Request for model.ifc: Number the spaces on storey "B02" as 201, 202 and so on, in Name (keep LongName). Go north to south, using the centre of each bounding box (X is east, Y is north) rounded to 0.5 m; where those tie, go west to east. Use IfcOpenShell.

First a look at what the model holds.

```python
import ifcopenshell
import ifcopenshell.util.element
import ifcopenshell.util.placement

model = ifcopenshell.open("model.ifc")
print(model.schema)
storey = next(s for s in model.by_type("IfcBuildingStorey") if s.Name == "B02")
spaces = [e for e in ifcopenshell.util.element.get_decomposition(storey) if e.is_a("IfcSpace")]
for e in sorted(spaces, key=lambda e: e.id()):
    origin = ifcopenshell.util.placement.get_local_placement(e.ObjectPlacement)[:3, 3]
    print(e.id(), e.Name, e.LongName, origin.round(2) + 0.0, sep=" | ")
```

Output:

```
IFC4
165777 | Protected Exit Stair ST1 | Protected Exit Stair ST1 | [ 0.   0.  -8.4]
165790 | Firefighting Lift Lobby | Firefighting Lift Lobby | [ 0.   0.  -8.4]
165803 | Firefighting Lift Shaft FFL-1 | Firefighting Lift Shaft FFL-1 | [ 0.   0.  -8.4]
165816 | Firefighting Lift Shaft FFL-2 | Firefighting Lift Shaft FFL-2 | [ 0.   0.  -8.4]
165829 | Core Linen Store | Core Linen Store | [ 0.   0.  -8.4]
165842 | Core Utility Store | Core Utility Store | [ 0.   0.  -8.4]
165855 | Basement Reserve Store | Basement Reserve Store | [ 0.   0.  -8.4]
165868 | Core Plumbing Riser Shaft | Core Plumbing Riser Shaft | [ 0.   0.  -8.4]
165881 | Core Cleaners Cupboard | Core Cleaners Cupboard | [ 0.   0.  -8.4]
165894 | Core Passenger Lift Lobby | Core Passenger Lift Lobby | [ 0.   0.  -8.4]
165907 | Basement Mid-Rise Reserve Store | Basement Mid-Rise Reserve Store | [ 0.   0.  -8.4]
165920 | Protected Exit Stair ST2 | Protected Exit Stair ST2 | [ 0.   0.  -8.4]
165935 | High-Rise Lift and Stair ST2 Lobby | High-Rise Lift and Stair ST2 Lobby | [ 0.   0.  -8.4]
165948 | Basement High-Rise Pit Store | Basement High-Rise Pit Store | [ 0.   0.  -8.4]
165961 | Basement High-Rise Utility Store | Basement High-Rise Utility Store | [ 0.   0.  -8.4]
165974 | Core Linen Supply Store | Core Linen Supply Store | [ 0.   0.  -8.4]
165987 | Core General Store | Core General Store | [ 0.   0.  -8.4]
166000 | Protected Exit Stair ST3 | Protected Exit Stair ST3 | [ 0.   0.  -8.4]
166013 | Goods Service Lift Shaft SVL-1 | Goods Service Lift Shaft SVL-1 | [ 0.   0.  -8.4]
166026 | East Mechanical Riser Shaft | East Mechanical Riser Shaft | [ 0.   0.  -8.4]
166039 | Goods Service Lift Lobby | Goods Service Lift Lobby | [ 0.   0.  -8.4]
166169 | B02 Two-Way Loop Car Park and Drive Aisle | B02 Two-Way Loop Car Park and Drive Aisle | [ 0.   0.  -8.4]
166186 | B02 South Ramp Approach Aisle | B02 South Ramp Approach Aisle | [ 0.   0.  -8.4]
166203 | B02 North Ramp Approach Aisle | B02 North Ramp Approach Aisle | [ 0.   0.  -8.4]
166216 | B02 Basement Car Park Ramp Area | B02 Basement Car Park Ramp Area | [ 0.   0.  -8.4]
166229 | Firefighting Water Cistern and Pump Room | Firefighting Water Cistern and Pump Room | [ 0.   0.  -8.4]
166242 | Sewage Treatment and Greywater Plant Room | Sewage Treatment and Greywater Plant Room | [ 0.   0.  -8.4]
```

```python
import ifcopenshell
import ifcopenshell.geom
import ifcopenshell.util.element
import ifcopenshell.util.shape

model = ifcopenshell.open("model.ifc")
settings = ifcopenshell.geom.settings()
settings.set("use-world-coords", True)


def centre(element):
    shape = ifcopenshell.geom.create_shape(settings, element)
    return ifcopenshell.util.shape.get_bbox_centroid(shape.geometry)


storey = next(s for s in model.by_type("IfcBuildingStorey") if s.Name == "B02")
spaces = [e for e in ifcopenshell.util.element.get_decomposition(storey) if e.is_a("IfcSpace")]

# Insertion points can sit at a corner or the storey origin, so sort by the geometry (in metres).
centres = {e: centre(e) for e in spaces}
spaces.sort(key=lambda e: (-round(centres[e][1] / 0.5), centres[e][0]))

for i, e in enumerate(spaces, start=1):
    number = f"2{i:02d}"
    e.Name = number
    print(e.id(), number)

model.write("model-out.ifc")
```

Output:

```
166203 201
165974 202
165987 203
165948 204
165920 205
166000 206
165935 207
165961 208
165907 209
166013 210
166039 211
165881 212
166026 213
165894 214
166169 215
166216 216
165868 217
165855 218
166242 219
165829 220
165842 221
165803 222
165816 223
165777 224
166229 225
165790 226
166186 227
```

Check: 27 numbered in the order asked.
